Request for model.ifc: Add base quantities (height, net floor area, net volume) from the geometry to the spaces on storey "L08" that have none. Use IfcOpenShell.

First a look at what the model holds.

```python
import ifcopenshell
import ifcopenshell.util.element
import ifcopenshell.util.unit

model = ifcopenshell.open("model.ifc")
print(model.schema)
for unit_type in ("LENGTHUNIT", "AREAUNIT", "VOLUMEUNIT"):
    print(unit_type, ifcopenshell.util.unit.calculate_unit_scale(model, unit_type))
storey = next(s for s in model.by_type("IfcBuildingStorey") if s.Name == "L08")
spaces = [e for e in ifcopenshell.util.element.get_decomposition(storey) if e.is_a("IfcSpace")]
for e in sorted(spaces, key=lambda e: e.id()):
    print(e.id(), e.is_a(), e.Name, list(ifcopenshell.util.element.get_psets(e, qtos_only=True)), sep=" | ")
```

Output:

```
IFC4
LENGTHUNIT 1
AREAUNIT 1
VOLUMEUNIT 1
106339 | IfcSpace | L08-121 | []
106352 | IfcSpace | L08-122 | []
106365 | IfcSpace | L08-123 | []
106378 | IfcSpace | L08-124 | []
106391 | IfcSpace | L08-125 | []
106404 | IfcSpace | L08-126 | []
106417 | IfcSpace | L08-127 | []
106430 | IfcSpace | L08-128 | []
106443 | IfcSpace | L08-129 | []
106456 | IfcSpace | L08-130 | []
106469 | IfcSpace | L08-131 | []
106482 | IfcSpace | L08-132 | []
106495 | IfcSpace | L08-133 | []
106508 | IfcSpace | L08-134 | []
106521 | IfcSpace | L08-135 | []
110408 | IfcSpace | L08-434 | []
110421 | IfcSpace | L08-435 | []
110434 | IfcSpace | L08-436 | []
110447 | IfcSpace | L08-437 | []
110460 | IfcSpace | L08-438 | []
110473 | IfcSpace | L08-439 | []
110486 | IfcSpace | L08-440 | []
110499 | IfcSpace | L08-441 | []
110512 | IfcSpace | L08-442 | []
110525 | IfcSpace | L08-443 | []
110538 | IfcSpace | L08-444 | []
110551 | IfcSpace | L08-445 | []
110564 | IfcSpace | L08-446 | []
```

```python
import ifcopenshell
import ifcopenshell.api.pset
import ifcopenshell.geom
import ifcopenshell.util.element
import ifcopenshell.util.shape
import ifcopenshell.util.unit

model = ifcopenshell.open("model.ifc")
unit_scale = ifcopenshell.util.unit.calculate_unit_scale(model)
area_scale = ifcopenshell.util.unit.calculate_unit_scale(model, "AREAUNIT")
volume_scale = ifcopenshell.util.unit.calculate_unit_scale(model, "VOLUMEUNIT")
settings = ifcopenshell.geom.settings()

storey = next(s for s in model.by_type("IfcBuildingStorey") if s.Name == "L08")
spaces = [e for e in ifcopenshell.util.element.get_decomposition(storey) if e.is_a("IfcSpace")]

for e in sorted(spaces, key=lambda e: e.id()):
    if ifcopenshell.util.element.get_psets(e, qtos_only=True, should_inherit=False):
        continue
    # Geometry comes back in metres, in the element's own axes.
    shape = ifcopenshell.geom.create_shape(settings, e)
    values = {
        "Height": ifcopenshell.util.shape.get_z(shape.geometry) / unit_scale,
        "NetFloorArea": ifcopenshell.util.shape.get_footprint_area(shape.geometry) / area_scale,
        "NetVolume": ifcopenshell.util.shape.get_volume(shape.geometry) / volume_scale,
    }
    qto = ifcopenshell.api.pset.add_qto(model, product=e, name="Qto_SpaceBaseQuantities")
    ifcopenshell.api.pset.edit_qto(model, qto=qto, properties=values)
    print(e.id(), {k: round(v, 3) for k, v in values.items()})

model.write("model_updated.ifc")
```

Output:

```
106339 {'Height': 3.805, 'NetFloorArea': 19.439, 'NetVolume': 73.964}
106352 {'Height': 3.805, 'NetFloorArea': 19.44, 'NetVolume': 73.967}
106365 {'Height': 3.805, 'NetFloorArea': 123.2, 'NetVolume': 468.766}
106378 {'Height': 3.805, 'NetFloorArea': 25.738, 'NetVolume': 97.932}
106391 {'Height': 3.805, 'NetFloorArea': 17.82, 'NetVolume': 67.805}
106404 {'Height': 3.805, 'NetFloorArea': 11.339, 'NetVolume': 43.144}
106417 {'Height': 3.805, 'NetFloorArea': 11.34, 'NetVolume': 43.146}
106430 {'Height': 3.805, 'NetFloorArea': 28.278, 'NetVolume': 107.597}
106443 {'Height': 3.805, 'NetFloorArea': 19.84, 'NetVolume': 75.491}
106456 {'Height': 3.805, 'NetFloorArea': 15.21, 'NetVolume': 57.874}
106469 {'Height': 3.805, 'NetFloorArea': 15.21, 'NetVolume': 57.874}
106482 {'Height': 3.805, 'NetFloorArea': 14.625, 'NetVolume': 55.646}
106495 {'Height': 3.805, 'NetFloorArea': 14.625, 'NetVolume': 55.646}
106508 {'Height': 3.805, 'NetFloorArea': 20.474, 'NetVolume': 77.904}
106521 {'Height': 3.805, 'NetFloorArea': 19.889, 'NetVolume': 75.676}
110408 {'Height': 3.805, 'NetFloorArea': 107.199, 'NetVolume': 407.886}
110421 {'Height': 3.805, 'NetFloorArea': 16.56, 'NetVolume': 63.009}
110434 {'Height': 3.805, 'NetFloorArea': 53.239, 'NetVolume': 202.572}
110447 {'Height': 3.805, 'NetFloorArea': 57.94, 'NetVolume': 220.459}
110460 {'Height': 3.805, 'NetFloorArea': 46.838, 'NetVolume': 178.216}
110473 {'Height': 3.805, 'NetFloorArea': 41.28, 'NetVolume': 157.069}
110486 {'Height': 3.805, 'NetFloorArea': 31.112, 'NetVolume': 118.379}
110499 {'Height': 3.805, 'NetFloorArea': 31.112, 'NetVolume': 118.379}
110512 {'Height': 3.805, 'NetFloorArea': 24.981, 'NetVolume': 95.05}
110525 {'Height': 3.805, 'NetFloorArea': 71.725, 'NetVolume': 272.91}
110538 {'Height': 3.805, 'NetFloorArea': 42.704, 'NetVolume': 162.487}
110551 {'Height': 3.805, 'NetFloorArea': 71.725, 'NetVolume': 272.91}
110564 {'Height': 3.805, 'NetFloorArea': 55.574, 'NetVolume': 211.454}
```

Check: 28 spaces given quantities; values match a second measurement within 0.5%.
